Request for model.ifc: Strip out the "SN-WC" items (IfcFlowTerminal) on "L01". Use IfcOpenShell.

First a look at what the model holds.

```python
import ifcopenshell
import ifcopenshell.util.element

model = ifcopenshell.open("model.ifc")
print(model.schema)
storey = next(s for s in model.by_type("IfcBuildingStorey") if s.Name == "L01")
terminals = [e for e in ifcopenshell.util.element.get_decomposition(storey) if e.is_a("IfcFlowTerminal")]
seen = {}
for e in terminals:
    element_type = ifcopenshell.util.element.get_type(e)
    name = element_type.Name if element_type not in (None, e) else None
    seen[name] = seen.get(name, 0) + 1
for name, count in sorted(seen.items(), key=str):
    print(count, "x", name)
```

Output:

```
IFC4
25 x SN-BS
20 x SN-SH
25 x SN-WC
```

```python
import ifcopenshell
import ifcopenshell.api.root
import ifcopenshell.util.element

model = ifcopenshell.open("model.ifc")

storey = next(s for s in model.by_type("IfcBuildingStorey") if s.Name == "L01")
terminals = [e for e in ifcopenshell.util.element.get_decomposition(storey) if e.is_a("IfcFlowTerminal")]
targets = [e for e in terminals if (t := ifcopenshell.util.element.get_type(e)) not in (None, e) and t.Name == "SN-WC"]

for e in targets:
    ifcopenshell.api.root.remove_product(model, product=e)
print(len(targets), "removed")

model.write("model-out.ifc")
```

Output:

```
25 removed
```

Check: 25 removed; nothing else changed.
